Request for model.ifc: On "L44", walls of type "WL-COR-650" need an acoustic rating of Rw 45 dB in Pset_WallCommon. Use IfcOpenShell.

First a look at what the model holds.

```python
import ifcopenshell
import ifcopenshell.util.element

model = ifcopenshell.open("model.ifc")
print(model.schema)
storey = next(s for s in model.by_type("IfcBuildingStorey") if s.Name == "L44")
walls = [e for e in ifcopenshell.util.element.get_decomposition(storey) if e.is_a("IfcWall")]
seen = {}
for e in walls:
    element_type = ifcopenshell.util.element.get_type(e)
    key = (element_type.Name if element_type != e and element_type else None, ifcopenshell.util.element.get_pset(e, "Pset_WallCommon", "AcousticRating"))
    seen[key] = seen.get(key, 0) + 1
for (name, value), count in sorted(seen.items(), key=str):
    print(count, "x", name, "|", value)
```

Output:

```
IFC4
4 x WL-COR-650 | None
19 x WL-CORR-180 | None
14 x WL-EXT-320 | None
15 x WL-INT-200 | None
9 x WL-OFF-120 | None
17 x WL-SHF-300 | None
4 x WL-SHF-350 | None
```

```python
import ifcopenshell
import ifcopenshell.api.pset
import ifcopenshell.util.element

model = ifcopenshell.open("model.ifc")

storey = next(s for s in model.by_type("IfcBuildingStorey") if s.Name == "L44")
walls = [e for e in ifcopenshell.util.element.get_decomposition(storey) if e.is_a("IfcWall")]

count = 0
for e in walls:
    element_type = ifcopenshell.util.element.get_type(e)
    if element_type in (None, e) or element_type.Name != "WL-COR-650":
        continue
    found = ifcopenshell.util.element.get_pset(e, "Pset_WallCommon", should_inherit=False)
    if found:
        pset = model.by_id(found["id"])
        if len(ifcopenshell.util.element.get_elements_by_pset(pset)) > 1:
            pset = ifcopenshell.api.pset.unshare_pset(model, products=[e], pset=pset)[0]
    else:
        pset = ifcopenshell.api.pset.add_pset(model, product=e, name="Pset_WallCommon")
    ifcopenshell.api.pset.edit_pset(model, pset=pset, properties={"AcousticRating": "Rw 45 dB"})
    count += 1

print(count, "walls updated")

model.write("model-out.ifc")
```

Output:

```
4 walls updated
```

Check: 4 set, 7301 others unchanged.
